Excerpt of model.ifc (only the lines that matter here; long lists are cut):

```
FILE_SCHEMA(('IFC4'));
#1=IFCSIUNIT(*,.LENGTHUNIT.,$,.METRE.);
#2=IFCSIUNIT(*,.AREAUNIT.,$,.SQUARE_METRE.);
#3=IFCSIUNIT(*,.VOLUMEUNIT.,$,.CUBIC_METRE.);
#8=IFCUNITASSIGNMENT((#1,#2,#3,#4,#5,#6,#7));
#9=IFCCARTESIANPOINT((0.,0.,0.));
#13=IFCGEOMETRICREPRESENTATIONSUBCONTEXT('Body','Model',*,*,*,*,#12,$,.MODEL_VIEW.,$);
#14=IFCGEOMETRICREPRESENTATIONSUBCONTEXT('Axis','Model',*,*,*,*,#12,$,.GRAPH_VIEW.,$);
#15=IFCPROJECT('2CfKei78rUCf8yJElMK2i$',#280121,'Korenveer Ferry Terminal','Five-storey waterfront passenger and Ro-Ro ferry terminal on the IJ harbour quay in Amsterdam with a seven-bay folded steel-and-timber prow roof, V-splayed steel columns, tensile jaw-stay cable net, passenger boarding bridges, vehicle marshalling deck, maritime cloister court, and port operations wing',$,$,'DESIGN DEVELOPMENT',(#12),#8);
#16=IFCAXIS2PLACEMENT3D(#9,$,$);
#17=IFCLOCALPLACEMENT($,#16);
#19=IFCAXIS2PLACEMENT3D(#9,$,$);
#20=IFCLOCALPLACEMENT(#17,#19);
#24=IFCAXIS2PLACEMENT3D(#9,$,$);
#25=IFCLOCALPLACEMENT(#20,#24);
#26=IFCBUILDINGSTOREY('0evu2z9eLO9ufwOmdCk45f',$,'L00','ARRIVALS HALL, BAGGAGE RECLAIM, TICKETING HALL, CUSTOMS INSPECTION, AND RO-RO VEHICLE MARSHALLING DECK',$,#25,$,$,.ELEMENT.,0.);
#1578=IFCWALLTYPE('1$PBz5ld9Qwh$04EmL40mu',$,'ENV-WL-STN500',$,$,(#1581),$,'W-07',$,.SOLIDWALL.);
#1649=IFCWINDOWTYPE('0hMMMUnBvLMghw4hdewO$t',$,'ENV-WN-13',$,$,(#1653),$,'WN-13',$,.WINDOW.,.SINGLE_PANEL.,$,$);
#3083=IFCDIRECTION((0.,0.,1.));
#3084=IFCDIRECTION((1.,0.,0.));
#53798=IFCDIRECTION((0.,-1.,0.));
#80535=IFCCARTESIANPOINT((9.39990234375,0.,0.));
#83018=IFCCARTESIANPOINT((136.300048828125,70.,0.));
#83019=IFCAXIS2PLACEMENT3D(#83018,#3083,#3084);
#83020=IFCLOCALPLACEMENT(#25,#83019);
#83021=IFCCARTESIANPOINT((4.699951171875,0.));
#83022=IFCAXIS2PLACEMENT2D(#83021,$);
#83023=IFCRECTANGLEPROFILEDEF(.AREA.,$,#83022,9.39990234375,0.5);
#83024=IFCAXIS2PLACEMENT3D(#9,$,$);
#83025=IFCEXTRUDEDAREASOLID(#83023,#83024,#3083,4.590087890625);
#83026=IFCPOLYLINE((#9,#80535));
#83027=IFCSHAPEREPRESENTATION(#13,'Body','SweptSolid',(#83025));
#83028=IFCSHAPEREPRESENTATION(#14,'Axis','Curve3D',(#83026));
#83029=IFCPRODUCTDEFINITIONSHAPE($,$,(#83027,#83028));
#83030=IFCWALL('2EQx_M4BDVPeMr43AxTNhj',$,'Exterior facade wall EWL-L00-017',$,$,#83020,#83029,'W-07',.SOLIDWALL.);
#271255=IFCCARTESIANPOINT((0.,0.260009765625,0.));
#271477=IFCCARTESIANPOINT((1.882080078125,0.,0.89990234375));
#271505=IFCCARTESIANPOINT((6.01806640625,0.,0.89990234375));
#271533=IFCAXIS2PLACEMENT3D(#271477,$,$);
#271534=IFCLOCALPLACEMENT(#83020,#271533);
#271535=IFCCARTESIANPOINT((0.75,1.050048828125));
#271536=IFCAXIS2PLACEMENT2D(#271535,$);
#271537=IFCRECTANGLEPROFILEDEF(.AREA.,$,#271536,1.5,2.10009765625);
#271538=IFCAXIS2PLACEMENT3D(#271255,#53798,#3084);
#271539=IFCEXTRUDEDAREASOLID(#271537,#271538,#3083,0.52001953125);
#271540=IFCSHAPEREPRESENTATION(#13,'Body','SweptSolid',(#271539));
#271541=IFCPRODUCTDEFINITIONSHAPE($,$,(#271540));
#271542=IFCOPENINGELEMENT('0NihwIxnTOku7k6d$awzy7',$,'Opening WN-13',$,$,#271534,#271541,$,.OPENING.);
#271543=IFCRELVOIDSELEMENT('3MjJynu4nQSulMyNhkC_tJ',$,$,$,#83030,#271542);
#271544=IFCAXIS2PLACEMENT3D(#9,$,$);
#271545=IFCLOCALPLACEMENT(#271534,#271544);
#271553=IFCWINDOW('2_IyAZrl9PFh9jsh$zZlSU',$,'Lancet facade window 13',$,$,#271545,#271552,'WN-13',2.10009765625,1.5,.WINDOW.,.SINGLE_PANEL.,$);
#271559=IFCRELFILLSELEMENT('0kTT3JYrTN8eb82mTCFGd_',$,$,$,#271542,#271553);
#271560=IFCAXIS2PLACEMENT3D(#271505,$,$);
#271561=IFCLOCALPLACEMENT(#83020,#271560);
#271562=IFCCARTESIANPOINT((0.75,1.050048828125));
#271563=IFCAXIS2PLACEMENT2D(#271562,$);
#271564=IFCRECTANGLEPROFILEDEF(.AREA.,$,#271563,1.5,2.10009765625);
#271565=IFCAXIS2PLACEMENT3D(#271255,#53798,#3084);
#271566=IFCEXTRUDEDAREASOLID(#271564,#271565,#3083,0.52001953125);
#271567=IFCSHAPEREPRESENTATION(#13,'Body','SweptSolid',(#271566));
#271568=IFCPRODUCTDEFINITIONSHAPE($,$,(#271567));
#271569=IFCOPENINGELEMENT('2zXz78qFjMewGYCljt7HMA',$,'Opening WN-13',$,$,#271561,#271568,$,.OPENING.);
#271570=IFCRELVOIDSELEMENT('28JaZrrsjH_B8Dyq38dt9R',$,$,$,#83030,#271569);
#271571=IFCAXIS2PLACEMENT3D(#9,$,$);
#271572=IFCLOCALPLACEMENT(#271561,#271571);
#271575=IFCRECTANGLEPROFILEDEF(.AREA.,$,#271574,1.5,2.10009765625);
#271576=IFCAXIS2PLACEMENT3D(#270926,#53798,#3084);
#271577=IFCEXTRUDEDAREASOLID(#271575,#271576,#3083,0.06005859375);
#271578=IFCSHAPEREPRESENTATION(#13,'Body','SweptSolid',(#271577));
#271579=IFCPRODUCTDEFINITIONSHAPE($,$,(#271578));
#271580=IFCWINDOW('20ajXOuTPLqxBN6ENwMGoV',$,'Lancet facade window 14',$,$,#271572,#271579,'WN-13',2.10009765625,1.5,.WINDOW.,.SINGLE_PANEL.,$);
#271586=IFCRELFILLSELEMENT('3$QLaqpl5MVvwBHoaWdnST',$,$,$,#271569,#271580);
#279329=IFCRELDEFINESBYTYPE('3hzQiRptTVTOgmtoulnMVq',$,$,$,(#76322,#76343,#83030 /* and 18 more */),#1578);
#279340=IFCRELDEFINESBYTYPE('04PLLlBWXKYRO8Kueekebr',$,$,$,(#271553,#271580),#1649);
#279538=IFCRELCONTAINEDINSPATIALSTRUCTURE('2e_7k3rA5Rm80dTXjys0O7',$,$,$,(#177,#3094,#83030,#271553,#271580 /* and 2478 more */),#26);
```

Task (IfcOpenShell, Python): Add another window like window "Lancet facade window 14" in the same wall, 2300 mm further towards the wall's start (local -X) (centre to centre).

```python
import ifcopenshell
import ifcopenshell.api.feature
import ifcopenshell.api.geometry
import ifcopenshell.api.root
import ifcopenshell.geom
import ifcopenshell.util.element
import ifcopenshell.util.placement
import ifcopenshell.util.shape
import ifcopenshell.util.unit

model = ifcopenshell.open("model.ifc")
unit_scale = ifcopenshell.util.unit.calculate_unit_scale(model)
settings = ifcopenshell.geom.settings()


def volume(element):
    """Net volume in cubic metres, openings subtracted."""
    shape = ifcopenshell.geom.create_shape(settings, element)
    return ifcopenshell.util.shape.get_volume(shape.geometry)


window = model.by_guid("20ajXOuTPLqxBN6ENwMGoV")
opening = window.FillsVoids[0].RelatingOpeningElement
wall = opening.VoidsElements[0].RelatingBuildingElement
before = volume(wall)
shift = ifcopenshell.util.placement.get_local_placement(wall.ObjectPlacement)[:3, 0] * -2.3 / unit_scale

# copy_class copies the void relationship, type, container and properties, but no geometry.
new_opening = ifcopenshell.api.root.copy_class(model, product=opening)
new_opening.Representation = ifcopenshell.util.element.copy_deep(
    model, opening.Representation, exclude=["IfcGeometricRepresentationContext", "IfcRepresentationMap"]
)
new_window = ifcopenshell.api.root.copy_class(model, product=window)
new_window.Representation = ifcopenshell.util.element.copy_deep(
    model, window.Representation, exclude=["IfcGeometricRepresentationContext", "IfcRepresentationMap"]
)
new_window.Tag = None
ifcopenshell.api.feature.add_filling(model, opening=new_opening, element=new_window)

for old, new in ((opening, new_opening), (window, new_window)):
    matrix = ifcopenshell.util.placement.get_local_placement(old.ObjectPlacement)
    matrix[:3, 3] += shift
    ifcopenshell.api.geometry.edit_object_placement(model, product=new, matrix=matrix, is_si=False)

after = volume(wall)

print(f"wall volume {before:.3f} -> {after:.3f} m3")

model.write("model_rev.ifc")
```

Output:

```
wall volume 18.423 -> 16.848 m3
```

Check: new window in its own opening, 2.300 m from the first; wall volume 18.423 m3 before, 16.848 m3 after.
